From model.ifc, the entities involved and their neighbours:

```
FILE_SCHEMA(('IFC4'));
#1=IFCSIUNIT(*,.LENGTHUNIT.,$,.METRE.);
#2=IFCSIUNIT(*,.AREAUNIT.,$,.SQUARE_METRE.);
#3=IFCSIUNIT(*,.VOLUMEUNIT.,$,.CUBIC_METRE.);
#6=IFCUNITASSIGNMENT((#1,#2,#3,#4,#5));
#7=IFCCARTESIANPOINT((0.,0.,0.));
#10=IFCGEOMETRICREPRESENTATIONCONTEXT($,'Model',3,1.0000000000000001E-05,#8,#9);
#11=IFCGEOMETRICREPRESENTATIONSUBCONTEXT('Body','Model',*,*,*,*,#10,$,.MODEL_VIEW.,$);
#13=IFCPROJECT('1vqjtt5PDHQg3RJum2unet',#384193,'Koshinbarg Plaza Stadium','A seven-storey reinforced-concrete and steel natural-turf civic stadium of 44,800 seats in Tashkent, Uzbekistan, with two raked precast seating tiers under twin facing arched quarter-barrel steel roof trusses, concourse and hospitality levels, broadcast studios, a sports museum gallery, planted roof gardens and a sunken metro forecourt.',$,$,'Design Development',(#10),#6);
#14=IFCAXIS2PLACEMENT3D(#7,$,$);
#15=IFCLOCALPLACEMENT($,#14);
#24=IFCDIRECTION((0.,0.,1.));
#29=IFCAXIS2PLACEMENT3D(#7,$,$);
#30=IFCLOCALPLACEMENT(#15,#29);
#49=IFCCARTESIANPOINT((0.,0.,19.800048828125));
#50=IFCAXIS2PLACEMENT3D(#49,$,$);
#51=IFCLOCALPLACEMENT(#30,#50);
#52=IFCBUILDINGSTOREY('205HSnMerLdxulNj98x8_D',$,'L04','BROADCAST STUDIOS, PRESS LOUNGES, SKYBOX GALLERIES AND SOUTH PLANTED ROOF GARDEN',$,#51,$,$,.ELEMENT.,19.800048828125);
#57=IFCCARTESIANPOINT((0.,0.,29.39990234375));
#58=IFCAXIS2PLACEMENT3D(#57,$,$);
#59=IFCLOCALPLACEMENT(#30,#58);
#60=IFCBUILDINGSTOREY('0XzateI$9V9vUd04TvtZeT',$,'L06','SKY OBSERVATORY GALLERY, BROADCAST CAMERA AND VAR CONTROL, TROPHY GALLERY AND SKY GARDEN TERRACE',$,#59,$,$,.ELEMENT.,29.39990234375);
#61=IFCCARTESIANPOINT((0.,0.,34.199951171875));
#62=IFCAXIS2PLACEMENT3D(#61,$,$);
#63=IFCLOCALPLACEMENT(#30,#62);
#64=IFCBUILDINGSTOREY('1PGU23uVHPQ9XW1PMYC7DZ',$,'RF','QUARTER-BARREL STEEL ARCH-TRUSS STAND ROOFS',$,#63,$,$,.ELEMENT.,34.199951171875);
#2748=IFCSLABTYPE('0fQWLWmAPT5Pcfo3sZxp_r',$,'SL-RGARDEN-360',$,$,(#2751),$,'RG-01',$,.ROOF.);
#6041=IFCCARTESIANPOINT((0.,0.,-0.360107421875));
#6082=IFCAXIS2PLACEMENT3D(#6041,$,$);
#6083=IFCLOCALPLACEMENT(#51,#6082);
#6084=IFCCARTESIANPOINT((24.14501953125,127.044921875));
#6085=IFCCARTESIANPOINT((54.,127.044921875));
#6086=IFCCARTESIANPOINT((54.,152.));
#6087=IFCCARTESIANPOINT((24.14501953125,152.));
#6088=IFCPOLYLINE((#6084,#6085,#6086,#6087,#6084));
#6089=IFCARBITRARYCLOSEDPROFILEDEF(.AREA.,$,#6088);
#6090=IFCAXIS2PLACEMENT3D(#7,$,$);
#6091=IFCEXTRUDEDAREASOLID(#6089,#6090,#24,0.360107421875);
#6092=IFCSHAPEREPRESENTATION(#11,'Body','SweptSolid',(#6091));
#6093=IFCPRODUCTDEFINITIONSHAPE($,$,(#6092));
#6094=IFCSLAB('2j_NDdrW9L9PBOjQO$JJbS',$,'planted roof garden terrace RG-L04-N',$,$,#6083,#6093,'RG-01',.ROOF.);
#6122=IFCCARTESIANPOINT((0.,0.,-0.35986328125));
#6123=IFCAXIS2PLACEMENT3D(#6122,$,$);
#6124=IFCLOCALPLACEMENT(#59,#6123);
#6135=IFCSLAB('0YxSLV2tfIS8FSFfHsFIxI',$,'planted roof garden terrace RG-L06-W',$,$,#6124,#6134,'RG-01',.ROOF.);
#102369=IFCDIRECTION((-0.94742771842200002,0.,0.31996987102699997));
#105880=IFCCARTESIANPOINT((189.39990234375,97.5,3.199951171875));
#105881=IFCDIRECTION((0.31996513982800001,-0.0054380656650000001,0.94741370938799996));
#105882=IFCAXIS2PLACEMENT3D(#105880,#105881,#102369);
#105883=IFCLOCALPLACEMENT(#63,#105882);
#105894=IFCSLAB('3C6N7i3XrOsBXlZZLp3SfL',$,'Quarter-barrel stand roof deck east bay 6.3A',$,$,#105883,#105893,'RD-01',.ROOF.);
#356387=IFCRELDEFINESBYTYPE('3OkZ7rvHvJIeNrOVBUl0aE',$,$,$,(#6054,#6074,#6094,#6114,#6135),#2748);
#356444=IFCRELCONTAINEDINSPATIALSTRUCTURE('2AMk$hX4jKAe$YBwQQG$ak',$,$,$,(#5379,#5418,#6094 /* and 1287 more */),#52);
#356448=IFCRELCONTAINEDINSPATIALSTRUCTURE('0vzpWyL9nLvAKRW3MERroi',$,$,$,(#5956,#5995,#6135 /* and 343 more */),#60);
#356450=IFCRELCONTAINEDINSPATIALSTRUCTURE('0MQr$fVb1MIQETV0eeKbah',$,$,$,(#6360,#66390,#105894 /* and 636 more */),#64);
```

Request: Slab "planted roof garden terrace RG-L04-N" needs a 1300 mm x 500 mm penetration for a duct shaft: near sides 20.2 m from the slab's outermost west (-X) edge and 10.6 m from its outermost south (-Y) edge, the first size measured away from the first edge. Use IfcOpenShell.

```python
import numpy as np
import ifcopenshell
import ifcopenshell.api.feature
import ifcopenshell.api.geometry
import ifcopenshell.api.root
import ifcopenshell.geom
import ifcopenshell.util.placement
import ifcopenshell.util.representation
import ifcopenshell.util.shape
import ifcopenshell.util.unit

model = ifcopenshell.open("model.ifc")
unit_scale = ifcopenshell.util.unit.calculate_unit_scale(model)
settings = ifcopenshell.geom.settings()


def volume(element):
    """Net volume in cubic metres, openings subtracted."""
    shape = ifcopenshell.geom.create_shape(settings, element)
    return ifcopenshell.util.shape.get_volume(shape.geometry)


slab = model.by_guid("2j_NDdrW9L9PBOjQO$JJbS")
before = volume(slab)

# Extent in the slab's own axes, in metres. The edges named are its -X and -Y sides.
slab_shape = ifcopenshell.geom.create_shape(settings, slab)
vertices = ifcopenshell.util.shape.get_vertices(slab_shape.geometry)
x_min, y_min, bottom = vertices.min(axis=0)
top = vertices[:, 2].max()

opening = ifcopenshell.api.root.create_entity(model, ifc_class="IfcOpeningElement", name="Duct shaft opening", predefined_type="OPENING")
context = ifcopenshell.util.representation.get_context(model, "Model", "Body", "MODEL_VIEW")
width, depth = 1.3, 0.5
outline = [(0.0, 0.0), (width, 0.0), (width, depth), (0.0, depth), (0.0, 0.0)]
# Overshoot both faces by 50 mm so the cut is clean.
shape = ifcopenshell.api.geometry.add_slab_representation(
    model, context=context, depth=top - bottom + 0.1, polyline=outline
)
ifcopenshell.api.geometry.assign_representation(model, product=opening, representation=shape)

matrix = ifcopenshell.util.placement.get_local_placement(slab.ObjectPlacement)
matrix[:, 3] = matrix @ np.append(np.array([x_min + 20.2, y_min + 10.6, bottom - 0.05]) / unit_scale, 1.0)
ifcopenshell.api.geometry.edit_object_placement(model, product=opening, matrix=matrix, is_si=False)
ifcopenshell.api.feature.add_feature(model, feature=opening, element=slab)

after = volume(slab)

print(f"slab volume {before:.3f} -> {after:.3f} m3")

model.write("model_edited.ifc")
```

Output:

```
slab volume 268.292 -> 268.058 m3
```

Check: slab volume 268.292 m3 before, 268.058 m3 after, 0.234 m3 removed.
